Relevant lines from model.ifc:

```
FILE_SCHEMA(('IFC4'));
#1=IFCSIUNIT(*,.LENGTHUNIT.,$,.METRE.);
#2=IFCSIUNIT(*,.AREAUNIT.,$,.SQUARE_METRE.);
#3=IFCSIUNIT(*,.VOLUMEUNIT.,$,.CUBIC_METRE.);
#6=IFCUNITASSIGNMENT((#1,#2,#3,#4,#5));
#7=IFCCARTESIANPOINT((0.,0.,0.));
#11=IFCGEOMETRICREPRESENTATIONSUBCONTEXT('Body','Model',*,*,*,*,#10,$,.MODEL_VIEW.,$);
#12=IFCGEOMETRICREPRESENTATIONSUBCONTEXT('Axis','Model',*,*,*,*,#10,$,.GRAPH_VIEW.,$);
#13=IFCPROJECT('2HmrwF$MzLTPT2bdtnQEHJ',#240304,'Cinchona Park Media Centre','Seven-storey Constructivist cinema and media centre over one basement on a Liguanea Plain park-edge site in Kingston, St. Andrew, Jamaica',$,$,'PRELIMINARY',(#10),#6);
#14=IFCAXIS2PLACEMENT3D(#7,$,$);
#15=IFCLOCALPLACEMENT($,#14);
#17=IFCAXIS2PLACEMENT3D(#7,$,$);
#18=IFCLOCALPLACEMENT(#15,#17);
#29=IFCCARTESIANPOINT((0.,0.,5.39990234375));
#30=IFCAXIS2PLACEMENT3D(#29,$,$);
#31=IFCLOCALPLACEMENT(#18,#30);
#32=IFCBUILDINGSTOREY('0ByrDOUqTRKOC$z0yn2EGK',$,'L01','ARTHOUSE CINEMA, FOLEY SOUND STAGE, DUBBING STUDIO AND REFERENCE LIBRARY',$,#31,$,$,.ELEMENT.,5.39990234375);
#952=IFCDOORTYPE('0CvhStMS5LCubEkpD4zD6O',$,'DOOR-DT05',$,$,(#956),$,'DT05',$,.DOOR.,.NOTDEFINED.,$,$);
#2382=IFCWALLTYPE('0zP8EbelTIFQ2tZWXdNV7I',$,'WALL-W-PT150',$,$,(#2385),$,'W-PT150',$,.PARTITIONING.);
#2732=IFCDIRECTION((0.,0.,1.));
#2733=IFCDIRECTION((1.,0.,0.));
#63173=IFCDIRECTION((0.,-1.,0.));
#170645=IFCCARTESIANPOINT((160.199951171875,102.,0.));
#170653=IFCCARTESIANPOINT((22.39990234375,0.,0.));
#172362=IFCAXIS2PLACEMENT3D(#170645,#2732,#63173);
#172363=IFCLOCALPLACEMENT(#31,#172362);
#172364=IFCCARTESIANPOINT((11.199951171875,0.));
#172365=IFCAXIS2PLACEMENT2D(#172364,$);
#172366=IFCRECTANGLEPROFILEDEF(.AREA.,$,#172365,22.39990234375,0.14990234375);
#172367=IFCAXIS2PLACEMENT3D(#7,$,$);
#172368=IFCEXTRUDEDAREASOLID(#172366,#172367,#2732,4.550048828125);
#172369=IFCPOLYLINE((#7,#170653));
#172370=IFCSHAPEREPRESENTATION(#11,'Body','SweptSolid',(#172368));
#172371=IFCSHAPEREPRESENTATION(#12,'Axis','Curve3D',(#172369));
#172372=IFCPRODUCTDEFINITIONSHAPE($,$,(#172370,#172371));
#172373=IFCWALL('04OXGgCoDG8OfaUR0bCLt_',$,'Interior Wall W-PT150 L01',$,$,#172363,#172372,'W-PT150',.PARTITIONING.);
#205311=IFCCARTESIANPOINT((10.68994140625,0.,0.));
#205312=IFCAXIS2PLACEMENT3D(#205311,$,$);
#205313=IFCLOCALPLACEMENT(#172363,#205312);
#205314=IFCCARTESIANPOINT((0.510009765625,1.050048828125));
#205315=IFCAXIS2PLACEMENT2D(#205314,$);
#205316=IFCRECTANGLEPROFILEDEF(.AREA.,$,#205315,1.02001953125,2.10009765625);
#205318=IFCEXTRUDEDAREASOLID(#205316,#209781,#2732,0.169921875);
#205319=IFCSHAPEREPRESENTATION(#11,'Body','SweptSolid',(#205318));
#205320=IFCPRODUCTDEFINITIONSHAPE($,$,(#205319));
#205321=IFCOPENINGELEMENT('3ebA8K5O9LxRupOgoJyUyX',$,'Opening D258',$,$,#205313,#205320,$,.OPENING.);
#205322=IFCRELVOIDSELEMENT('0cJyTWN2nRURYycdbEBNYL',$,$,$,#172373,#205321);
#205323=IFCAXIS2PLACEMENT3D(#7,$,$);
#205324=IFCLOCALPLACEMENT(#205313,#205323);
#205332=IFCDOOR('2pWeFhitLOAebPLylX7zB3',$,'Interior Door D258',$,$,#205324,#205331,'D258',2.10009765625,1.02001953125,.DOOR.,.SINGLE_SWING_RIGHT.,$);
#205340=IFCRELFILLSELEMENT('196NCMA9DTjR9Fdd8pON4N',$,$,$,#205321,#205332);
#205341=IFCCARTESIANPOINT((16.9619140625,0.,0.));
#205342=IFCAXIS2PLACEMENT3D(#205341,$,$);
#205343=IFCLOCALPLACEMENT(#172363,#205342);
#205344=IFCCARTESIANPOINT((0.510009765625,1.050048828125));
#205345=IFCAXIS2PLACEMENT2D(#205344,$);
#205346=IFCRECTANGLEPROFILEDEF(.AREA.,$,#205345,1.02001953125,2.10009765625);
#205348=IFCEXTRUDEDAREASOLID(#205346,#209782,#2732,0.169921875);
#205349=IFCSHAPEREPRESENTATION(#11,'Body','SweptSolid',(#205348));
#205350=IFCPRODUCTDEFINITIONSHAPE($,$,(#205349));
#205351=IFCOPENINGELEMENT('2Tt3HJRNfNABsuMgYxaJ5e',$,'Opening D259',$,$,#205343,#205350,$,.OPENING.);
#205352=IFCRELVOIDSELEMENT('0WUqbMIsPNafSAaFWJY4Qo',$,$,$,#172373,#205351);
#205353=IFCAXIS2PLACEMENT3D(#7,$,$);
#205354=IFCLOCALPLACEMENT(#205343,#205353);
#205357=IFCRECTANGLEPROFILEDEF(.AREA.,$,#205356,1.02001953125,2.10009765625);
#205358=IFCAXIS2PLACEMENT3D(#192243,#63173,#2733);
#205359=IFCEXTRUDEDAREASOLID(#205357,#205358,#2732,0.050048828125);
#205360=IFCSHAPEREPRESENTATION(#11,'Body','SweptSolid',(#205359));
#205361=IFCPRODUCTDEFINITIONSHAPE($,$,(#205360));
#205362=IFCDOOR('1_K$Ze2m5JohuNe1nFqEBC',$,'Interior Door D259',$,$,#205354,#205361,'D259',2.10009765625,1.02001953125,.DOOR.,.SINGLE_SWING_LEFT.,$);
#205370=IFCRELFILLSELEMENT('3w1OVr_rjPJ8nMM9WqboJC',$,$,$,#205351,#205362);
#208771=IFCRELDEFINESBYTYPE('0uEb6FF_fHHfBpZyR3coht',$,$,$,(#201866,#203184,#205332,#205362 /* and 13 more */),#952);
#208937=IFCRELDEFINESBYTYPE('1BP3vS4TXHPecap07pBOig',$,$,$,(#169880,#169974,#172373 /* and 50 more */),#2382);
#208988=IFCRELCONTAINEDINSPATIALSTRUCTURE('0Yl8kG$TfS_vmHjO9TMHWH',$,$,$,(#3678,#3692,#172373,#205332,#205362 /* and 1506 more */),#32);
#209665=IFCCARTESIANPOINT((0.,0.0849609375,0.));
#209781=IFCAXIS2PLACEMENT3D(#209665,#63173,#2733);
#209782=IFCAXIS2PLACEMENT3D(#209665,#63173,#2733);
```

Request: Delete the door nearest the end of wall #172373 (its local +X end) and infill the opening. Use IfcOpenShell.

```python
import ifcopenshell
import ifcopenshell.api.feature
import ifcopenshell.api.root
import ifcopenshell.geom
import ifcopenshell.util.shape

model = ifcopenshell.open("model.ifc")
settings = ifcopenshell.geom.settings()


def volume(element):
    """Net volume in cubic metres, openings subtracted."""
    shape = ifcopenshell.geom.create_shape(settings, element)
    return ifcopenshell.util.shape.get_volume(shape.geometry)


door = model.by_guid("1_K$Ze2m5JohuNe1nFqEBC")
opening = door.FillsVoids[0].RelatingOpeningElement
wall = opening.VoidsElements[0].RelatingBuildingElement
before = volume(wall)

ifcopenshell.api.root.remove_product(model, product=door)
ifcopenshell.api.feature.remove_feature(model, feature=opening)

after = volume(wall)

print(f"wall volume {before:.3f} -> {after:.3f} m3")

model.write("model-out.ifc")
```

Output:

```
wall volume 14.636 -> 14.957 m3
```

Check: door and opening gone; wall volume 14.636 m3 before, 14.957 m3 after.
